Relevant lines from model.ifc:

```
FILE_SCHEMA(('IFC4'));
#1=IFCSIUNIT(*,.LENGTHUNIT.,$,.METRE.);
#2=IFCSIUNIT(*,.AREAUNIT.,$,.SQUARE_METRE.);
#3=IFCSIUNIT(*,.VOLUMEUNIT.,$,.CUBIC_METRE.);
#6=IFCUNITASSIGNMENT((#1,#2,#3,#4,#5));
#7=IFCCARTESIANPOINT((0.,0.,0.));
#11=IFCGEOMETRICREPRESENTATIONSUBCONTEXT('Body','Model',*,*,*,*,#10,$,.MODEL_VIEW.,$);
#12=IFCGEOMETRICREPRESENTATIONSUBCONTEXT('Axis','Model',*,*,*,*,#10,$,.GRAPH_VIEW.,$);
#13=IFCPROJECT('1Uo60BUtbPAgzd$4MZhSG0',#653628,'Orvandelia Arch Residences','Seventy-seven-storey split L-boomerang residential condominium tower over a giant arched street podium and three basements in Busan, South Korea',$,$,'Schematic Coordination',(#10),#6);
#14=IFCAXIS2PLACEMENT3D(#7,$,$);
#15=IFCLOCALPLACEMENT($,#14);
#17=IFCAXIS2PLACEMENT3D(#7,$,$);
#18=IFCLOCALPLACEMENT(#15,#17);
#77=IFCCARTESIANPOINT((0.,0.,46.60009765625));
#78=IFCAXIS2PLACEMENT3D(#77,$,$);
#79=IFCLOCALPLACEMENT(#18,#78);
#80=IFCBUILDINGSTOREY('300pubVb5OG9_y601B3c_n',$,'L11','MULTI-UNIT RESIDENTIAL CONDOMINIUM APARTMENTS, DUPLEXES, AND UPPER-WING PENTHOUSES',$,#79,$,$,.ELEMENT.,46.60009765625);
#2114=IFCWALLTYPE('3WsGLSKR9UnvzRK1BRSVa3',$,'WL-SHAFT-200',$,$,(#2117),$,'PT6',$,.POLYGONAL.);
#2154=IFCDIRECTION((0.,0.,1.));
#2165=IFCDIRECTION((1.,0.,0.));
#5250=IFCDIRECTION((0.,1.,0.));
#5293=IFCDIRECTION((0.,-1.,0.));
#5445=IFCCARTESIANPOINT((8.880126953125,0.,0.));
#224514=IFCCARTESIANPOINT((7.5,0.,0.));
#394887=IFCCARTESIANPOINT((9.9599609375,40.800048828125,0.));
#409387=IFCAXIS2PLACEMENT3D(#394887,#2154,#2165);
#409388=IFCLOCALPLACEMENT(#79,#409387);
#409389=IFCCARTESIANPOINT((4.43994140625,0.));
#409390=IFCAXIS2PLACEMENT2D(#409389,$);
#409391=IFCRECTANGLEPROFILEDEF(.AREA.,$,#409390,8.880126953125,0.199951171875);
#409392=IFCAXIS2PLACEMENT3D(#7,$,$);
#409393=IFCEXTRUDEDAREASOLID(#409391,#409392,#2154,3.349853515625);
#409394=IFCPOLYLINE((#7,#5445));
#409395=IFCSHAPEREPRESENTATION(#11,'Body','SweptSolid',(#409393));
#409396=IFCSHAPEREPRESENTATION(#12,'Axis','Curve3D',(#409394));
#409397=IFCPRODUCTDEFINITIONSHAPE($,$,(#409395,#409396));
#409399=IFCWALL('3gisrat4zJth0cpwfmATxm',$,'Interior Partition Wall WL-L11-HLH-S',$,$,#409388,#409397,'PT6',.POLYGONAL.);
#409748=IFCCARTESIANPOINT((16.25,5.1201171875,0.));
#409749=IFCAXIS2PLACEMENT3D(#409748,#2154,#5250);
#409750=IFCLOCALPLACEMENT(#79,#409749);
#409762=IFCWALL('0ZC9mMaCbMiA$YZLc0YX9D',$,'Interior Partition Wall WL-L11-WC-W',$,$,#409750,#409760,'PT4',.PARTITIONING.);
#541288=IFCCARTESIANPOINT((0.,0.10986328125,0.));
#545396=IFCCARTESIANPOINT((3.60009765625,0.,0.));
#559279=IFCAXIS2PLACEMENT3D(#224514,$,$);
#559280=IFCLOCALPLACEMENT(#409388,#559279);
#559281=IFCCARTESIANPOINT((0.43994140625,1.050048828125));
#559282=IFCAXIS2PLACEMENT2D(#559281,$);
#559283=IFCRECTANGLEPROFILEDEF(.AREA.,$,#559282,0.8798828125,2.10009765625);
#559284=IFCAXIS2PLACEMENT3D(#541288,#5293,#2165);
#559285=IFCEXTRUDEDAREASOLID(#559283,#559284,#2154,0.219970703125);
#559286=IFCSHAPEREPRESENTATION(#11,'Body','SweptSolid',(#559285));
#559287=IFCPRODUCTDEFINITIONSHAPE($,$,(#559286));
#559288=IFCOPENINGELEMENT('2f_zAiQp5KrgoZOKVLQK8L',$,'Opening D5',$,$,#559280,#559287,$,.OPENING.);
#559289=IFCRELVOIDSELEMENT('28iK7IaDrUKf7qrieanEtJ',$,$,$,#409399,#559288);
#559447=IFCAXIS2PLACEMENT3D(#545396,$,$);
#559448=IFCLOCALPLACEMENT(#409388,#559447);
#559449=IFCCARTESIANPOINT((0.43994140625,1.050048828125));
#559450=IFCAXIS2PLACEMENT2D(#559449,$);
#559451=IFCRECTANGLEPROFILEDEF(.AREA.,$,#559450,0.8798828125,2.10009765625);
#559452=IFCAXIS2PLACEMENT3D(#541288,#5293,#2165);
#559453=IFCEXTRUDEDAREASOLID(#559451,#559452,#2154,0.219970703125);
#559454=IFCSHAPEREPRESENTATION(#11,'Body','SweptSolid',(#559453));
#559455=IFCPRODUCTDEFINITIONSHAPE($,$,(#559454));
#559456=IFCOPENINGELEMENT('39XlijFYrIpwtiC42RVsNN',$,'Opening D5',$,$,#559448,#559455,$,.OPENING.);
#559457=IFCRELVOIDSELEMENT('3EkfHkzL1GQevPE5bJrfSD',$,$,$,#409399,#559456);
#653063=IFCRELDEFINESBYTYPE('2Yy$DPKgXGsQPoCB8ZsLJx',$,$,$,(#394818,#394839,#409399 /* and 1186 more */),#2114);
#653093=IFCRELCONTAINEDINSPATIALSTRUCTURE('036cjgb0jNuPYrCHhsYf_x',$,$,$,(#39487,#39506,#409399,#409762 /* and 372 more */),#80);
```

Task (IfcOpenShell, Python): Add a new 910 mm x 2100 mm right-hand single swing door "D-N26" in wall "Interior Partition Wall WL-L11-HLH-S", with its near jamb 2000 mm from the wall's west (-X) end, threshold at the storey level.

```python
import numpy as np
import ifcopenshell
import ifcopenshell.api.feature
import ifcopenshell.api.geometry
import ifcopenshell.api.root
import ifcopenshell.api.spatial
import ifcopenshell.geom
import ifcopenshell.util.element
import ifcopenshell.util.placement
import ifcopenshell.util.representation
import ifcopenshell.util.shape
import ifcopenshell.util.unit

model = ifcopenshell.open("model.ifc")
unit_scale = ifcopenshell.util.unit.calculate_unit_scale(model)
settings = ifcopenshell.geom.settings()


def volume(element):
    """Net volume in cubic metres, openings subtracted."""
    shape = ifcopenshell.geom.create_shape(settings, element)
    return ifcopenshell.util.shape.get_volume(shape.geometry)


wall = model.by_id(409399)
storey = ifcopenshell.util.element.get_container(wall, ifc_class="IfcBuildingStorey")
context = ifcopenshell.util.representation.get_context(model, "Model", "Body", "MODEL_VIEW")
before = volume(wall)

width, height, from_end, sill = 0.91, 2.1, 2, 0.0  # metres

# The wall runs along its own X axis, and the end named is its -X end.
wall_shape = ifcopenshell.geom.create_shape(settings, wall)
x, y, z = ifcopenshell.util.shape.get_vertices(wall_shape.geometry).T
start = x.min() + from_end
face, thickness = float(y.min()), float(y.max() - y.min())
wall_matrix = ifcopenshell.util.placement.get_local_placement(wall.ObjectPlacement)
level = ifcopenshell.util.placement.get_local_placement(storey.ObjectPlacement)[2, 3]


def in_wall(x, y):
    """Placement at x, y metres in the wall's axes, at sill height."""
    matrix = wall_matrix.copy()
    matrix[:, 3] = wall_matrix @ np.array([x / unit_scale, y / unit_scale, 0.0, 1.0])
    matrix[2, 3] = level + sill / unit_scale
    return matrix


# Opening: a box that overshoots both wall faces by 50 mm.
opening = ifcopenshell.api.root.create_entity(model, ifc_class="IfcOpeningElement", predefined_type="OPENING")
box = ifcopenshell.api.geometry.add_wall_representation(
    model, context=context, length=width, height=height, thickness=thickness + 0.1
)
ifcopenshell.api.geometry.assign_representation(model, product=opening, representation=box)
ifcopenshell.api.geometry.edit_object_placement(model, product=opening, matrix=in_wall(start, face - 0.05), is_si=False)
ifcopenshell.api.feature.add_feature(model, feature=opening, element=wall)

door = ifcopenshell.api.root.create_entity(model, ifc_class="IfcDoor", name="D-N26", predefined_type="DOOR")
door.OverallWidth, door.OverallHeight = width / unit_scale, height / unit_scale
door.OperationType = "SINGLE_SWING_RIGHT"
body = ifcopenshell.api.geometry.add_door_representation(
    model,
    context=context,
    overall_width=door.OverallWidth,
    overall_height=door.OverallHeight,
    operation_type="SINGLE_SWING_RIGHT",
    lining_properties={"LiningDepth": thickness / unit_scale, "ThresholdDepth": thickness / unit_scale},
)
ifcopenshell.api.geometry.assign_representation(model, product=door, representation=body)
ifcopenshell.api.spatial.assign_container(model, products=[door], relating_structure=storey)
ifcopenshell.api.feature.add_filling(model, opening=opening, element=door)

# The lining spans the wall, so the door starts at the wall face.
ifcopenshell.api.geometry.edit_object_placement(model, product=door, matrix=in_wall(start, face), is_si=False)

after = volume(wall)

print(f"wall volume {before:.3f} -> {after:.3f} m3")

model.write("model_v2.ifc")
```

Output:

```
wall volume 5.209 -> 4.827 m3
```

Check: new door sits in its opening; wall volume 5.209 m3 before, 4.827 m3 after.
